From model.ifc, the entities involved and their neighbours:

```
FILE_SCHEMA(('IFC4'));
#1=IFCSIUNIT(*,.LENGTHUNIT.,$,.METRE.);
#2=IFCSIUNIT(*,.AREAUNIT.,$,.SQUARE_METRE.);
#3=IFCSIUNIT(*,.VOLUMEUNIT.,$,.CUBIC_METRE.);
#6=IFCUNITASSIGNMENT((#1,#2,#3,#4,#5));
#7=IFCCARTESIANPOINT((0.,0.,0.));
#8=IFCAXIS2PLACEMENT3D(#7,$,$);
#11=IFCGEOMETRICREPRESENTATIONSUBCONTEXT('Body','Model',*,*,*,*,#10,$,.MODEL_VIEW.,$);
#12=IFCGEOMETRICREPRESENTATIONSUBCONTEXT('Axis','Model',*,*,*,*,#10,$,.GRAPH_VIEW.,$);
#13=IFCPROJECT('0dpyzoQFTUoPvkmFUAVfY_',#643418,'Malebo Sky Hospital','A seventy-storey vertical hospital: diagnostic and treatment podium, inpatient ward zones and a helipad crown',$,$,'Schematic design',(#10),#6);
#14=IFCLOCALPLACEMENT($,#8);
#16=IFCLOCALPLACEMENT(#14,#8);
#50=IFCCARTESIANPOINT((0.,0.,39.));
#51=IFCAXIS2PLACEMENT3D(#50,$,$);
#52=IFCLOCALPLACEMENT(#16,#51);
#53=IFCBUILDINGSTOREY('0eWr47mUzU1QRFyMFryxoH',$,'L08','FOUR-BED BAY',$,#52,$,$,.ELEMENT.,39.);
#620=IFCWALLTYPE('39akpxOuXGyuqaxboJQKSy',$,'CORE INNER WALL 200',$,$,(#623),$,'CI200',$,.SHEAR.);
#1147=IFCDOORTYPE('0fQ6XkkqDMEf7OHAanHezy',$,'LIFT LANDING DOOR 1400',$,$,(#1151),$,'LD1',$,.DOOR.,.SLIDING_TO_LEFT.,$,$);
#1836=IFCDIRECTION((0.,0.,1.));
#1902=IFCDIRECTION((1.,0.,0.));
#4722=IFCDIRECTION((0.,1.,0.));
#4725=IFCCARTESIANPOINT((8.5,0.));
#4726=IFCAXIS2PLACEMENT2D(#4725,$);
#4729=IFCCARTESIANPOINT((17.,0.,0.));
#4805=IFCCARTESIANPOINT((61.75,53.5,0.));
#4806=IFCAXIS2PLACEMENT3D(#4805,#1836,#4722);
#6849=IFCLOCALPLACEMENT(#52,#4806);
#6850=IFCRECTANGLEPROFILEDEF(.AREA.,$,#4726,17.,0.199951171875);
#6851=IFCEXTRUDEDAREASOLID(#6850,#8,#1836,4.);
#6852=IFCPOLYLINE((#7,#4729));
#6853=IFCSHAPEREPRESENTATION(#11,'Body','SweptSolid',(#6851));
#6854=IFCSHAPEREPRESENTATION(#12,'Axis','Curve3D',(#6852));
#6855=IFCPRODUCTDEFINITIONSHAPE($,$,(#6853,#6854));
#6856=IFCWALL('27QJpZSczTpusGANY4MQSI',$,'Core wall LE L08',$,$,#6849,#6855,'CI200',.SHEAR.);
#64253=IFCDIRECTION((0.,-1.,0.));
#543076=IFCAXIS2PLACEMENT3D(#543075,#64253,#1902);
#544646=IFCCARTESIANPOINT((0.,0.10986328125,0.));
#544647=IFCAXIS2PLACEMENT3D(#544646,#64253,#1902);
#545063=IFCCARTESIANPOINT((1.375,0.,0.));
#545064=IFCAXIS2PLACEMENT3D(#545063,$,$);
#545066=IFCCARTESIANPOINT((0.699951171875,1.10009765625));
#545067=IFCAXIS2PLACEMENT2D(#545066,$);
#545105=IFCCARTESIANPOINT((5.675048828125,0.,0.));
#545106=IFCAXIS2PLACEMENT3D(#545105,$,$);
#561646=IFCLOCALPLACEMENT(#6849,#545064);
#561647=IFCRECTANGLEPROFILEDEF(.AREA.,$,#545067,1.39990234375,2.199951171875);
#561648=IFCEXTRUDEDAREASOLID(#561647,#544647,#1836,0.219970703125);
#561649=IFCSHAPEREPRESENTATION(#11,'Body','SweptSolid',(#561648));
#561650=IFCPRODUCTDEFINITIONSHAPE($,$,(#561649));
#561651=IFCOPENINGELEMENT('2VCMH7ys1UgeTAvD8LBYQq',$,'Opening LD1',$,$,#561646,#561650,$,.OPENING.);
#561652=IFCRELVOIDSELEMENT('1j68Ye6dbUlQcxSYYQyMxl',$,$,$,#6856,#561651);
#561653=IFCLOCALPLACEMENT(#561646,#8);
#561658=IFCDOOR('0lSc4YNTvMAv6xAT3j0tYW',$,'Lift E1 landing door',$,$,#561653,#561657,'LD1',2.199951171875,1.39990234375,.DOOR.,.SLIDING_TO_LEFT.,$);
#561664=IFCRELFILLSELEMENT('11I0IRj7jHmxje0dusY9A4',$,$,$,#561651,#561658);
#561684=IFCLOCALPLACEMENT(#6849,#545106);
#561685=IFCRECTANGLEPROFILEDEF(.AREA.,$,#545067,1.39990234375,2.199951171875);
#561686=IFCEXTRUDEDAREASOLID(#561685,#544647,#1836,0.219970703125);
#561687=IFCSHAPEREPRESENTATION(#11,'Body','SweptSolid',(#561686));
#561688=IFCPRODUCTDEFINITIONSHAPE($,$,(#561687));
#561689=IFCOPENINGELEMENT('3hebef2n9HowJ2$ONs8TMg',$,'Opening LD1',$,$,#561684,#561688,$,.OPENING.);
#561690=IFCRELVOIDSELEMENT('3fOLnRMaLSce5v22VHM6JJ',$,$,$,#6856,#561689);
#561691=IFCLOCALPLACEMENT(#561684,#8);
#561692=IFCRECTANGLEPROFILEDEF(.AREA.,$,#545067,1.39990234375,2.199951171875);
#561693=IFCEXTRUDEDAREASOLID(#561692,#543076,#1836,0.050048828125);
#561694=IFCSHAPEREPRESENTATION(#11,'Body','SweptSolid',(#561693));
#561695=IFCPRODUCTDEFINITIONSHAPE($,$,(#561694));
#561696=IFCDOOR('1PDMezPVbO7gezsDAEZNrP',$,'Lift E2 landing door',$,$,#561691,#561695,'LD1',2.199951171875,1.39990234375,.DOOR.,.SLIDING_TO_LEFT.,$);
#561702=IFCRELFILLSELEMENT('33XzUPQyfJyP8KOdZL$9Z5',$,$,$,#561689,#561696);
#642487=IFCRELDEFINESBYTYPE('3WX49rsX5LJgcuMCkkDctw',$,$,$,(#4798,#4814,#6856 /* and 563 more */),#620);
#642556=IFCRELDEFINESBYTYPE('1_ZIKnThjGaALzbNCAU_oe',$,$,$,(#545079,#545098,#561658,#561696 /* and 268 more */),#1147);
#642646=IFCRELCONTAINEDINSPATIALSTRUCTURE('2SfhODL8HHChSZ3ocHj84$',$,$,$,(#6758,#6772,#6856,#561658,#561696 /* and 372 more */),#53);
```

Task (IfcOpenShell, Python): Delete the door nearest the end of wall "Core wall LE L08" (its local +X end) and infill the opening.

```python
import ifcopenshell
import ifcopenshell.api.feature
import ifcopenshell.api.root
import ifcopenshell.geom
import ifcopenshell.util.shape

model = ifcopenshell.open("model.ifc")
settings = ifcopenshell.geom.settings()


def volume(element):
    """Net volume in cubic metres, openings subtracted."""
    shape = ifcopenshell.geom.create_shape(settings, element)
    return ifcopenshell.util.shape.get_volume(shape.geometry)


door = model.by_guid("1PDMezPVbO7gezsDAEZNrP")
opening = door.FillsVoids[0].RelatingOpeningElement
wall = opening.VoidsElements[0].RelatingBuildingElement
before = volume(wall)

ifcopenshell.api.root.remove_product(model, product=door)
ifcopenshell.api.feature.remove_feature(model, feature=opening)

after = volume(wall)

print(f"wall volume {before:.3f} -> {after:.3f} m3")

model.write("model-out.ifc")
```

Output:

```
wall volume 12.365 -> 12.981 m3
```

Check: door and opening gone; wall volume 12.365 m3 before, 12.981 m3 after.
